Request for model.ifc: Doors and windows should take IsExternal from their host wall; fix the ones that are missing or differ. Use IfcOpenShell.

First a look at what the model holds.

```python
import ifcopenshell
import ifcopenshell.util.element

model = ifcopenshell.open("model.ifc")
print(model.schema)
seen = {}
for e in model.by_type("IfcDoor") + model.by_type("IfcWindow"):
    if not e.FillsVoids:
        continue
    host = e.FillsVoids[0].RelatingOpeningElement.VoidsElements[0].RelatingBuildingElement
    own = ifcopenshell.util.element.get_pset(e, f"Pset_{e.is_a()[3:].removesuffix('StandardCase')}Common", "IsExternal")
    wall = ifcopenshell.util.element.get_pset(host, "Pset_WallCommon", "IsExternal")
    seen[e.is_a(), own, wall] = seen.get((e.is_a(), own, wall), 0) + 1
for (cls, own, wall), count in sorted(seen.items(), key=str):
    print(count, cls, "IsExternal:", own, "| host wall:", wall)
```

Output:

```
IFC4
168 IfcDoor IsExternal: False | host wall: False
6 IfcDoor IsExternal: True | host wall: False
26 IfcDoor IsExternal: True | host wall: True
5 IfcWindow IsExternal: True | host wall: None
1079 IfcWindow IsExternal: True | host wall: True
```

```python
import ifcopenshell
import ifcopenshell.api.pset
import ifcopenshell.util.element

model = ifcopenshell.open("model.ifc")

count = 0
for ifc_class, pset_name in (("IfcDoor", "Pset_DoorCommon"), ("IfcWindow", "Pset_WindowCommon")):
    for e in model.by_type(ifc_class):
        if not e.FillsVoids:
            continue
        host = e.FillsVoids[0].RelatingOpeningElement.VoidsElements[0].RelatingBuildingElement
        external = ifcopenshell.util.element.get_pset(host, "Pset_WallCommon", "IsExternal")
        if external is None or ifcopenshell.util.element.get_pset(e, pset_name, "IsExternal") == external:
            continue
        pset = ifcopenshell.api.pset.add_pset(model, product=e, name=pset_name)
        ifcopenshell.api.pset.edit_pset(model, pset=pset, properties={"IsExternal": external})
        count += 1

print(count, "updated")

model.write("model_edited.ifc")
```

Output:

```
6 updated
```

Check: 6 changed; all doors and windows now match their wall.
